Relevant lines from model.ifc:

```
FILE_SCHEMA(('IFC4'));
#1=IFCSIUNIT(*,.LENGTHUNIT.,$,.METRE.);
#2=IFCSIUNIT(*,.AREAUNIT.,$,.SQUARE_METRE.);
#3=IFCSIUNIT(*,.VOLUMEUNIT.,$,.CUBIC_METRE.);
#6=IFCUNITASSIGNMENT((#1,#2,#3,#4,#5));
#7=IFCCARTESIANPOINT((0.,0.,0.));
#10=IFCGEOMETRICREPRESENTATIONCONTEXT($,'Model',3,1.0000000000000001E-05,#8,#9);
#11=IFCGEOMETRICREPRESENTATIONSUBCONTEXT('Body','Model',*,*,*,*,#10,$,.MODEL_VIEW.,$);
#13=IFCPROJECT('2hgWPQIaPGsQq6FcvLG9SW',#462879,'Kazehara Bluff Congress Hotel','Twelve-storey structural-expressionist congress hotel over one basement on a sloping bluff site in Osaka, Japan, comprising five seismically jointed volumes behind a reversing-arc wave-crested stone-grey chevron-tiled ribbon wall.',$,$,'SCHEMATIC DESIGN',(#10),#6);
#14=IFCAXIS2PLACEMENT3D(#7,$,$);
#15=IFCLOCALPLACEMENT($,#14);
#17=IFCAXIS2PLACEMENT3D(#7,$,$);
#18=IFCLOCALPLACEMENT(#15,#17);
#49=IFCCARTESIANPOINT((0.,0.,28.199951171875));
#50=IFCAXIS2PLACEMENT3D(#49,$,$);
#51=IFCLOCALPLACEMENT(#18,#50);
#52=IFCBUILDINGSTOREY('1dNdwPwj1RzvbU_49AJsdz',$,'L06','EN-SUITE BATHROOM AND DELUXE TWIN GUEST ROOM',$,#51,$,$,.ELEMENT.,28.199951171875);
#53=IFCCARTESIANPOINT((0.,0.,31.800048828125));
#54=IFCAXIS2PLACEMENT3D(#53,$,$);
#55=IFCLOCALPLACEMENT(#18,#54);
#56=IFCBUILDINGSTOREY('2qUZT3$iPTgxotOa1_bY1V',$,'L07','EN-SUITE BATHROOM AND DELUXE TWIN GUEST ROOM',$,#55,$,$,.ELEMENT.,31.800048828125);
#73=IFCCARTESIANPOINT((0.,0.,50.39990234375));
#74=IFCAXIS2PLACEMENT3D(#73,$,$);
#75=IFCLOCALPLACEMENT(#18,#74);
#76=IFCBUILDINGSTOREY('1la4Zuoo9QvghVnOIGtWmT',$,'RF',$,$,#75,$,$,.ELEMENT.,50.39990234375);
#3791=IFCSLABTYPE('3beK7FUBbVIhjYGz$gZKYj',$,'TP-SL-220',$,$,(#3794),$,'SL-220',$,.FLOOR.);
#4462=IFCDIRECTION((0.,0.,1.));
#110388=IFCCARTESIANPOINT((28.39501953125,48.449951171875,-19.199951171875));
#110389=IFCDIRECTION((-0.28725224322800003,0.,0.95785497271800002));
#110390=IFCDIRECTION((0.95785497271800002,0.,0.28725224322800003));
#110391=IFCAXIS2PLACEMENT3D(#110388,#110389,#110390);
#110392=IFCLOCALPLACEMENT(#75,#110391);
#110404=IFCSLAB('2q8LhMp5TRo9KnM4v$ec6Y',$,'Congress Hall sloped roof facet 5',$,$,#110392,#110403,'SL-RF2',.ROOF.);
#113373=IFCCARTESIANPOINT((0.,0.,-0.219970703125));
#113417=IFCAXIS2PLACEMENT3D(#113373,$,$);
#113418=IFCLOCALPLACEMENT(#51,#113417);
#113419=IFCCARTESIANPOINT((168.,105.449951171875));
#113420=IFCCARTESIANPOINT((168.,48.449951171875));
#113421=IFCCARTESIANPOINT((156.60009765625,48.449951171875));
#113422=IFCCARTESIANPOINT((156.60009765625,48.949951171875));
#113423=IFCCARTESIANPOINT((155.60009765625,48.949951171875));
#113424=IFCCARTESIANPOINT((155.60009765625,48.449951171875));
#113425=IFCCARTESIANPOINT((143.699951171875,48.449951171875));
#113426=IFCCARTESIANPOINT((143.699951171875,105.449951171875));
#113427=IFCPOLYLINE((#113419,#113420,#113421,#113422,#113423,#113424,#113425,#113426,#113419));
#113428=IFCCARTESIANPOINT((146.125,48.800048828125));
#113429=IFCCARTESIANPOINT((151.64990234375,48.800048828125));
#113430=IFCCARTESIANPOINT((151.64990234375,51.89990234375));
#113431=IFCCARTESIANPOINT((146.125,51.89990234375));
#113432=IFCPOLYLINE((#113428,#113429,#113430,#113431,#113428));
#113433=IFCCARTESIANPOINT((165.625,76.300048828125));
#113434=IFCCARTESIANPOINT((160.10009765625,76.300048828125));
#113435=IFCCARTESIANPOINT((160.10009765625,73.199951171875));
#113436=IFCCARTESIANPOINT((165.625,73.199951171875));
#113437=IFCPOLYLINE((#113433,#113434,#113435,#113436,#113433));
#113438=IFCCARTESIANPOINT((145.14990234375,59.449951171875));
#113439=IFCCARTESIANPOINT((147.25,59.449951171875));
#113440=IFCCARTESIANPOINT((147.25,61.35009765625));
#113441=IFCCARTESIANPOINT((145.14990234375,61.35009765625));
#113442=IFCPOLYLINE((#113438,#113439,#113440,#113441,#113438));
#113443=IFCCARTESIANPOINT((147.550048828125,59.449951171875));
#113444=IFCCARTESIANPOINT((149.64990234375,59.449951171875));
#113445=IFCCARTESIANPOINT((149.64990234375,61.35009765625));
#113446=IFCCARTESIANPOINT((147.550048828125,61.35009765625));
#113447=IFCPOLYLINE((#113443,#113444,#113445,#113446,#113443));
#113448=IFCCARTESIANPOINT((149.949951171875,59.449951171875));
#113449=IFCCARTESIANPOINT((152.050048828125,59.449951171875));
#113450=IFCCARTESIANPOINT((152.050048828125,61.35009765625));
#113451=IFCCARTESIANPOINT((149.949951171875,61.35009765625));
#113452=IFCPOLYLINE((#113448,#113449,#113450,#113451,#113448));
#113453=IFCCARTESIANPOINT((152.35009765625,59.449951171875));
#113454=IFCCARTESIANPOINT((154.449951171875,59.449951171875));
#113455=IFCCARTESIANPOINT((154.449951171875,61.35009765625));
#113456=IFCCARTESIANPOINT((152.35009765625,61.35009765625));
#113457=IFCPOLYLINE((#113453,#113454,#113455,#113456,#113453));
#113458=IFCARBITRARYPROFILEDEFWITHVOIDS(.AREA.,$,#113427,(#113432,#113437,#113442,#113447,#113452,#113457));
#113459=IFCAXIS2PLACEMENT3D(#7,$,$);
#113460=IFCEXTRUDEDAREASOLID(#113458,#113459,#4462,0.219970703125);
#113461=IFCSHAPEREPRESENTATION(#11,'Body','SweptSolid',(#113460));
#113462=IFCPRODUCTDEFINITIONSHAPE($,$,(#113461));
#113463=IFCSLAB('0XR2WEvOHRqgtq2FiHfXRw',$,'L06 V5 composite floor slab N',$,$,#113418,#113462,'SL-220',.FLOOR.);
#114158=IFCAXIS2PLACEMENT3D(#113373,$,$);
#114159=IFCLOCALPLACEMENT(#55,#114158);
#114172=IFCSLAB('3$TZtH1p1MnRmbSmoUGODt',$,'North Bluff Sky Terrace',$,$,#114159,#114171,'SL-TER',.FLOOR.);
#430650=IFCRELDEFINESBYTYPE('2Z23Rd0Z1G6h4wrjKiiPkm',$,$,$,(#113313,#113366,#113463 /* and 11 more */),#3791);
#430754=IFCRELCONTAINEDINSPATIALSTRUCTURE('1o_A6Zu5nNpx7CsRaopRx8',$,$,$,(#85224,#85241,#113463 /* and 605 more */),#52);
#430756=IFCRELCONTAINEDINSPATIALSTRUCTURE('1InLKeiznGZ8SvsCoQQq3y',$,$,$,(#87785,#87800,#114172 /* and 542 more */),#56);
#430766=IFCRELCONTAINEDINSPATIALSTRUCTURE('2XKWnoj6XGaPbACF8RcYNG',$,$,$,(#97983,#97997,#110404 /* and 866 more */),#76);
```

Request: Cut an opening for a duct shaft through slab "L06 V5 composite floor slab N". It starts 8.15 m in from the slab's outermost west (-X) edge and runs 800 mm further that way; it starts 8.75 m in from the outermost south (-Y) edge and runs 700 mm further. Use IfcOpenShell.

```python
import numpy as np
import ifcopenshell
import ifcopenshell.api.feature
import ifcopenshell.api.geometry
import ifcopenshell.api.root
import ifcopenshell.geom
import ifcopenshell.util.placement
import ifcopenshell.util.representation
import ifcopenshell.util.shape
import ifcopenshell.util.unit

model = ifcopenshell.open("model.ifc")
unit_scale = ifcopenshell.util.unit.calculate_unit_scale(model)
settings = ifcopenshell.geom.settings()


def volume(element):
    """Net volume in cubic metres, openings subtracted."""
    shape = ifcopenshell.geom.create_shape(settings, element)
    return ifcopenshell.util.shape.get_volume(shape.geometry)


slab = model.by_guid("0XR2WEvOHRqgtq2FiHfXRw")
before = volume(slab)

# Extent in the slab's own axes, in metres. The edges named are its -X and -Y sides.
slab_shape = ifcopenshell.geom.create_shape(settings, slab)
vertices = ifcopenshell.util.shape.get_vertices(slab_shape.geometry)
x_min, y_min, bottom = vertices.min(axis=0)
top = vertices[:, 2].max()

opening = ifcopenshell.api.root.create_entity(model, ifc_class="IfcOpeningElement", name="Duct shaft opening", predefined_type="OPENING")
context = ifcopenshell.util.representation.get_context(model, "Model", "Body", "MODEL_VIEW")
width, depth = 0.8, 0.7
outline = [(0.0, 0.0), (width, 0.0), (width, depth), (0.0, depth), (0.0, 0.0)]
# Overshoot both faces by 50 mm so the cut is clean.
shape = ifcopenshell.api.geometry.add_slab_representation(
    model, context=context, depth=top - bottom + 0.1, polyline=outline
)
ifcopenshell.api.geometry.assign_representation(model, product=opening, representation=shape)

matrix = ifcopenshell.util.placement.get_local_placement(slab.ObjectPlacement)
matrix[:, 3] = matrix @ np.append(np.array([x_min + 8.15, y_min + 8.75, bottom - 0.05]) / unit_scale, 1.0)
ifcopenshell.api.geometry.edit_object_placement(model, product=opening, matrix=matrix, is_si=False)
ifcopenshell.api.feature.add_feature(model, feature=opening, element=slab)

after = volume(slab)

print(f"slab volume {before:.3f} -> {after:.3f} m3")

model.write("model_updated.ifc")
```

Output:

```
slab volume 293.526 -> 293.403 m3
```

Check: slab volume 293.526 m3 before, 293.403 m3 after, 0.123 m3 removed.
